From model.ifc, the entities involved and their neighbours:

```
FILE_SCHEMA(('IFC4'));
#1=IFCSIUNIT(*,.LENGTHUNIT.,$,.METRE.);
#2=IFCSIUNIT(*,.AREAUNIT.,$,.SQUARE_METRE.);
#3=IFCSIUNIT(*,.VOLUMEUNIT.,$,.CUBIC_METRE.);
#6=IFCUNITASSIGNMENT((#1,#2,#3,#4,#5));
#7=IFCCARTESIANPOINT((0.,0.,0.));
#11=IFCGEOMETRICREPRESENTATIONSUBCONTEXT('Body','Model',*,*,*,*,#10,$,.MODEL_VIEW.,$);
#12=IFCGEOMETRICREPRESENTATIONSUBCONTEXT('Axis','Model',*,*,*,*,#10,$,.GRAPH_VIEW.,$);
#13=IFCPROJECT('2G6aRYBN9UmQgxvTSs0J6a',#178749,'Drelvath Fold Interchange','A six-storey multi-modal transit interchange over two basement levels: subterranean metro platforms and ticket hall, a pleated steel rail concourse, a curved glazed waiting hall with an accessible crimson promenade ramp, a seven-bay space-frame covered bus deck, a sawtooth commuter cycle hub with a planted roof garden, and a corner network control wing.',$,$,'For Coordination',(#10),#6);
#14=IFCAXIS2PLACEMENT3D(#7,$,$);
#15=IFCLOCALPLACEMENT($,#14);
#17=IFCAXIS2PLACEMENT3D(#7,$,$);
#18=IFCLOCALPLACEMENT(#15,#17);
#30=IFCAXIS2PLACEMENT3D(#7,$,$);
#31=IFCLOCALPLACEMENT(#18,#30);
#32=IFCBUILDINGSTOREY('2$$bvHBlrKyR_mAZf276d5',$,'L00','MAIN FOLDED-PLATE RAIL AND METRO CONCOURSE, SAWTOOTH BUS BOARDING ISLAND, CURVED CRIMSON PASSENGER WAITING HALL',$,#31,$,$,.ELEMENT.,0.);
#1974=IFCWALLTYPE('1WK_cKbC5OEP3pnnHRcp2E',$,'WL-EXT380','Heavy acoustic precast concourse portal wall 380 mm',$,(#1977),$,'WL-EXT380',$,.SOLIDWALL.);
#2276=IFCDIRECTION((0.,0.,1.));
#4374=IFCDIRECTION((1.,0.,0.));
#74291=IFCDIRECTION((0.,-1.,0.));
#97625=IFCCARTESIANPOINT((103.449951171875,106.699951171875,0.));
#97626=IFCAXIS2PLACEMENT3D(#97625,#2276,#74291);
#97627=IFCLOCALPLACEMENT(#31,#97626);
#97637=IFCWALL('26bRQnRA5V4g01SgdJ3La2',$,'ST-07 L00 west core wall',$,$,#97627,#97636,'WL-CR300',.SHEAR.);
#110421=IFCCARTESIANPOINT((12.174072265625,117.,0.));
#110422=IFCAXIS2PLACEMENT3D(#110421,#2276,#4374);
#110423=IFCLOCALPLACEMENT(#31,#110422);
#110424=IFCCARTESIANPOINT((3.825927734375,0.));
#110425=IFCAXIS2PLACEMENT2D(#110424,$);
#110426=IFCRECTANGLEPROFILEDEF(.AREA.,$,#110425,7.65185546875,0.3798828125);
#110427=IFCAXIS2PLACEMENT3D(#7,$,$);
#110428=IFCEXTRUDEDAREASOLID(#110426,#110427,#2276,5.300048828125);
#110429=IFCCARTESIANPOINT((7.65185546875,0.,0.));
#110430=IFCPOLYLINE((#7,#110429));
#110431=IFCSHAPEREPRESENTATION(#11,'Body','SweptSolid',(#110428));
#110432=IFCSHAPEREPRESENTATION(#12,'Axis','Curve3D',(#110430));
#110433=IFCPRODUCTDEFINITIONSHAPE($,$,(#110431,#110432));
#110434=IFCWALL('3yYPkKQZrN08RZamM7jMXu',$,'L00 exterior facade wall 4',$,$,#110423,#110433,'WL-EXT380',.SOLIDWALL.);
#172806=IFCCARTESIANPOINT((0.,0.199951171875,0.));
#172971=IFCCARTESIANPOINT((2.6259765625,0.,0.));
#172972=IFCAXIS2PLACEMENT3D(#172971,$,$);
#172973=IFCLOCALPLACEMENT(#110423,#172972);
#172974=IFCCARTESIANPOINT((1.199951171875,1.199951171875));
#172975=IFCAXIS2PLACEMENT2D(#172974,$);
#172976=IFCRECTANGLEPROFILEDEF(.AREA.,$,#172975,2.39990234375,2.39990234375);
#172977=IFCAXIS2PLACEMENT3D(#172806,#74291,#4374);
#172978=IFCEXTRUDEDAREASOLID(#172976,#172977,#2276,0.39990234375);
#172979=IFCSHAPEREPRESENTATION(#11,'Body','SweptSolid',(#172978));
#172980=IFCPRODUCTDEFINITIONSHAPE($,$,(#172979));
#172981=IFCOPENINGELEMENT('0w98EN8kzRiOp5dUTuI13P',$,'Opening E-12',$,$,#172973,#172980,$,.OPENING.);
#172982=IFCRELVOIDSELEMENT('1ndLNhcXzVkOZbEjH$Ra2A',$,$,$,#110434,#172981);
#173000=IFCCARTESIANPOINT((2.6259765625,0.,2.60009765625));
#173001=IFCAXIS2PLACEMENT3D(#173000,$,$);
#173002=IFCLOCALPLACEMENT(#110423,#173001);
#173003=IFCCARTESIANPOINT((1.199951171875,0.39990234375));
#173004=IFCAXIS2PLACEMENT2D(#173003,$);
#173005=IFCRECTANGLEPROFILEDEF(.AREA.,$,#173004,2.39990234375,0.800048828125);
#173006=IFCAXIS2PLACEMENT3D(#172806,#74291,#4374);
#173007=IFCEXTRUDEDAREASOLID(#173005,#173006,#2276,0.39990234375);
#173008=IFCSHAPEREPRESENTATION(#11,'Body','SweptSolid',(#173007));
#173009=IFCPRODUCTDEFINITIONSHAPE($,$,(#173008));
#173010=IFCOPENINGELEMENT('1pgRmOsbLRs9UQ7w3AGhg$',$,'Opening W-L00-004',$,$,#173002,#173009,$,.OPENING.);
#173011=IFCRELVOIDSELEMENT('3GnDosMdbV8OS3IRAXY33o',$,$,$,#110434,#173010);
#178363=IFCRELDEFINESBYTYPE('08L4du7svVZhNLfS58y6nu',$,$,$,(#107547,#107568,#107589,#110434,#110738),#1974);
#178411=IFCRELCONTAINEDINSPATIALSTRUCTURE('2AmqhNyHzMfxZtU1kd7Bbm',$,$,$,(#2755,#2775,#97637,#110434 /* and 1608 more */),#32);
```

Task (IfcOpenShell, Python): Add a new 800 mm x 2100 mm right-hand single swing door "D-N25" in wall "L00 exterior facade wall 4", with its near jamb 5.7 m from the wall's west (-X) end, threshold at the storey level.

```python
import numpy as np
import ifcopenshell
import ifcopenshell.api.feature
import ifcopenshell.api.geometry
import ifcopenshell.api.root
import ifcopenshell.api.spatial
import ifcopenshell.geom
import ifcopenshell.util.element
import ifcopenshell.util.placement
import ifcopenshell.util.representation
import ifcopenshell.util.shape
import ifcopenshell.util.unit

model = ifcopenshell.open("model.ifc")
unit_scale = ifcopenshell.util.unit.calculate_unit_scale(model)
settings = ifcopenshell.geom.settings()


def volume(element):
    """Net volume in cubic metres, openings subtracted."""
    shape = ifcopenshell.geom.create_shape(settings, element)
    return ifcopenshell.util.shape.get_volume(shape.geometry)


wall = model.by_guid("3yYPkKQZrN08RZamM7jMXu")
storey = ifcopenshell.util.element.get_container(wall, ifc_class="IfcBuildingStorey")
context = ifcopenshell.util.representation.get_context(model, "Model", "Body", "MODEL_VIEW")
before = volume(wall)

width, height, from_end, sill = 0.8, 2.1, 5.7, 0.0  # metres

# The wall runs along its own X axis, and the end named is its -X end.
wall_shape = ifcopenshell.geom.create_shape(settings, wall)
x, y, z = ifcopenshell.util.shape.get_vertices(wall_shape.geometry).T
start = x.min() + from_end
face, thickness = float(y.min()), float(y.max() - y.min())
wall_matrix = ifcopenshell.util.placement.get_local_placement(wall.ObjectPlacement)
level = ifcopenshell.util.placement.get_local_placement(storey.ObjectPlacement)[2, 3]


def in_wall(x, y):
    """Placement at x, y metres in the wall's axes, at sill height."""
    matrix = wall_matrix.copy()
    matrix[:, 3] = wall_matrix @ np.array([x / unit_scale, y / unit_scale, 0.0, 1.0])
    matrix[2, 3] = level + sill / unit_scale
    return matrix


# Opening: a box that overshoots both wall faces by 50 mm.
opening = ifcopenshell.api.root.create_entity(model, ifc_class="IfcOpeningElement", predefined_type="OPENING")
box = ifcopenshell.api.geometry.add_wall_representation(
    model, context=context, length=width, height=height, thickness=thickness + 0.1
)
ifcopenshell.api.geometry.assign_representation(model, product=opening, representation=box)
ifcopenshell.api.geometry.edit_object_placement(model, product=opening, matrix=in_wall(start, face - 0.05), is_si=False)
ifcopenshell.api.feature.add_feature(model, feature=opening, element=wall)

door = ifcopenshell.api.root.create_entity(model, ifc_class="IfcDoor", name="D-N25", predefined_type="DOOR")
door.OverallWidth, door.OverallHeight = width / unit_scale, height / unit_scale
door.OperationType = "SINGLE_SWING_RIGHT"
body = ifcopenshell.api.geometry.add_door_representation(
    model,
    context=context,
    overall_width=door.OverallWidth,
    overall_height=door.OverallHeight,
    operation_type="SINGLE_SWING_RIGHT",
    lining_properties={"LiningDepth": thickness / unit_scale, "ThresholdDepth": thickness / unit_scale},
)
ifcopenshell.api.geometry.assign_representation(model, product=door, representation=body)
ifcopenshell.api.spatial.assign_container(model, products=[door], relating_structure=storey)
ifcopenshell.api.feature.add_filling(model, opening=opening, element=door)

# The lining spans the wall, so the door starts at the wall face.
ifcopenshell.api.geometry.edit_object_placement(model, product=door, matrix=in_wall(start, face), is_si=False)

after = volume(wall)

print(f"wall volume {before:.3f} -> {after:.3f} m3")

model.write("model_rev.ifc")
```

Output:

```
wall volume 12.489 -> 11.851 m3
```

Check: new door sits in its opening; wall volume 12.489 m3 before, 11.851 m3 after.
